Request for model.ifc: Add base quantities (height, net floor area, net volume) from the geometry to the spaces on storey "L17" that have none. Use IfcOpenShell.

First a look at what the model holds.

```python
import ifcopenshell
import ifcopenshell.util.element
import ifcopenshell.util.unit

model = ifcopenshell.open("model.ifc")
print(model.schema)
for unit_type in ("LENGTHUNIT", "AREAUNIT", "VOLUMEUNIT"):
    print(unit_type, ifcopenshell.util.unit.calculate_unit_scale(model, unit_type))
storey = next(s for s in model.by_type("IfcBuildingStorey") if s.Name == "L17")
spaces = [e for e in ifcopenshell.util.element.get_decomposition(storey) if e.is_a("IfcSpace")]
for e in sorted(spaces, key=lambda e: e.id()):
    print(e.id(), e.is_a(), e.Name, list(ifcopenshell.util.element.get_psets(e, qtos_only=True)), sep=" | ")
```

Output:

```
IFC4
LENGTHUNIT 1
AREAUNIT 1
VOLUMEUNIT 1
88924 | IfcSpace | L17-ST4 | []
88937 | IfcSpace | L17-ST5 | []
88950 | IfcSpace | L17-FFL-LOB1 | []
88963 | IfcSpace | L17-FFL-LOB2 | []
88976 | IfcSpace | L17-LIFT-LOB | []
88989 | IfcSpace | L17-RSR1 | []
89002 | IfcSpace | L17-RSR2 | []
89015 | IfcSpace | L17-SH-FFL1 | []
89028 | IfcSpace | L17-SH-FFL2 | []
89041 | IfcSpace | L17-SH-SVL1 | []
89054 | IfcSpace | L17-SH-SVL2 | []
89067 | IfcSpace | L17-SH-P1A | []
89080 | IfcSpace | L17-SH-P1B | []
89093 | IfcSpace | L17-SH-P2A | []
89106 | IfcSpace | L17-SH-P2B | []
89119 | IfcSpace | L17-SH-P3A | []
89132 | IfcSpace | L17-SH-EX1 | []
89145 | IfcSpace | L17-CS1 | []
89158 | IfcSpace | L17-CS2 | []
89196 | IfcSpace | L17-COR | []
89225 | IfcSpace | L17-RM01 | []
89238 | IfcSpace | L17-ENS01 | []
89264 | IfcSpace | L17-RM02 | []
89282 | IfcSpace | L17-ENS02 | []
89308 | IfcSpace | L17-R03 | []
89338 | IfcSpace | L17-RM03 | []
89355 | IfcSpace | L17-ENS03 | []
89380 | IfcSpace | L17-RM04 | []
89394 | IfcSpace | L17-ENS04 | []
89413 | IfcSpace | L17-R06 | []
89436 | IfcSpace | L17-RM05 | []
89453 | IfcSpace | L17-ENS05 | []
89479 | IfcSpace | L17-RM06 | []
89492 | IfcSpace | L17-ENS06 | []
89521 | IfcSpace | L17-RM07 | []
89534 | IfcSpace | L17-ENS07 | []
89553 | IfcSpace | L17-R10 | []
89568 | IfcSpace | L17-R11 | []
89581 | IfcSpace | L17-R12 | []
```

```python
import ifcopenshell
import ifcopenshell.api.pset
import ifcopenshell.geom
import ifcopenshell.util.element
import ifcopenshell.util.shape
import ifcopenshell.util.unit

model = ifcopenshell.open("model.ifc")
unit_scale = ifcopenshell.util.unit.calculate_unit_scale(model)
area_scale = ifcopenshell.util.unit.calculate_unit_scale(model, "AREAUNIT")
volume_scale = ifcopenshell.util.unit.calculate_unit_scale(model, "VOLUMEUNIT")
settings = ifcopenshell.geom.settings()

storey = next(s for s in model.by_type("IfcBuildingStorey") if s.Name == "L17")
spaces = [e for e in ifcopenshell.util.element.get_decomposition(storey) if e.is_a("IfcSpace")]

for e in sorted(spaces, key=lambda e: e.id()):
    if ifcopenshell.util.element.get_psets(e, qtos_only=True, should_inherit=False):
        continue
    # Geometry comes back in metres, in the element's own axes.
    shape = ifcopenshell.geom.create_shape(settings, e)
    values = {
        "Height": ifcopenshell.util.shape.get_z(shape.geometry) / unit_scale,
        "NetFloorArea": ifcopenshell.util.shape.get_footprint_area(shape.geometry) / area_scale,
        "NetVolume": ifcopenshell.util.shape.get_volume(shape.geometry) / volume_scale,
    }
    qto = ifcopenshell.api.pset.add_qto(model, product=e, name="Qto_SpaceBaseQuantities")
    ifcopenshell.api.pset.edit_qto(model, qto=qto, properties=values)
    print(e.id(), {k: round(v, 3) for k, v in values.items()})

model.write("model_v2.ifc")
```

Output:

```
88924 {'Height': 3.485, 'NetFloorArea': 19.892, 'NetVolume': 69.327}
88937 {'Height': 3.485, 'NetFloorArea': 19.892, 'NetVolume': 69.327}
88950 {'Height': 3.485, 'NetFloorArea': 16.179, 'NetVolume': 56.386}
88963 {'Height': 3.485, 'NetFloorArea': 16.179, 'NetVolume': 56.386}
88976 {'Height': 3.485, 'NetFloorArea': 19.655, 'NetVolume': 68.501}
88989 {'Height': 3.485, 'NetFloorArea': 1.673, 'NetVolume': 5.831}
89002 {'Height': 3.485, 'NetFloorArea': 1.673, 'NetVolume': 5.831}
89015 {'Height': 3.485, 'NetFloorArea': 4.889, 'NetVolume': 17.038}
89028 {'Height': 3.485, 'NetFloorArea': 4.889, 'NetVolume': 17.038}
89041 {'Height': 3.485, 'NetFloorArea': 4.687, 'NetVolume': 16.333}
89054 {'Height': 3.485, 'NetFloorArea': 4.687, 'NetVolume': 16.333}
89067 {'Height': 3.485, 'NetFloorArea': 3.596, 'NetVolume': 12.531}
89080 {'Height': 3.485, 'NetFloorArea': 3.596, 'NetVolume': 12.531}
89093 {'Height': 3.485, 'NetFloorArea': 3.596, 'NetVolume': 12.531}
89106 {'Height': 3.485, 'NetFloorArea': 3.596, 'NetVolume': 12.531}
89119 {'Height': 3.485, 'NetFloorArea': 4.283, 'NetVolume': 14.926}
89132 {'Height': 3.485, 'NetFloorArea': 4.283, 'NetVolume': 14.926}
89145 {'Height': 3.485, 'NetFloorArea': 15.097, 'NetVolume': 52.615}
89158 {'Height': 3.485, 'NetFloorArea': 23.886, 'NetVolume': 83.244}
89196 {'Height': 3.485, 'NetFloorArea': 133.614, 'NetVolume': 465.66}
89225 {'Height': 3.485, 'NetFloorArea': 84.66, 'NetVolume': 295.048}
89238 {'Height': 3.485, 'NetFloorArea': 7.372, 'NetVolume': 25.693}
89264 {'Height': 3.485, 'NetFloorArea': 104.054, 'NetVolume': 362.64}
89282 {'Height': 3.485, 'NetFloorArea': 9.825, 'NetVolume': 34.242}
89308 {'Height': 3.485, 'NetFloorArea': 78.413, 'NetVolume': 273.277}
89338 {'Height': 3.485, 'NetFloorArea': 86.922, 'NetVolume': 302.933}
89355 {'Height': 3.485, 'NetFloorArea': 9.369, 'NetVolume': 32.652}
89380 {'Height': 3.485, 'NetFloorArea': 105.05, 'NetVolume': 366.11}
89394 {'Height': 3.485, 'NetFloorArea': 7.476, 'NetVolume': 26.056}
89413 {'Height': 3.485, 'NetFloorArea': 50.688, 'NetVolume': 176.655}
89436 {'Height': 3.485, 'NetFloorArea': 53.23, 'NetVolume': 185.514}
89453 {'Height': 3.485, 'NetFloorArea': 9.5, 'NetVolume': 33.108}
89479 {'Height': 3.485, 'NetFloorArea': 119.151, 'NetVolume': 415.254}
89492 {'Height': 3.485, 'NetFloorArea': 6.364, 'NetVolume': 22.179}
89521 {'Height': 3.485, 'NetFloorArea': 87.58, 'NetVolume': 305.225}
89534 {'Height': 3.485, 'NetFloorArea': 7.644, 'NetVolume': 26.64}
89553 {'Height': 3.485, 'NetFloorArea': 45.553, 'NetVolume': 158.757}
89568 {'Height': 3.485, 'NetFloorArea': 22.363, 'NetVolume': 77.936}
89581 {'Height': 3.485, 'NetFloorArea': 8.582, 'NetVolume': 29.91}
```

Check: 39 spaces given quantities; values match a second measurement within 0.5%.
